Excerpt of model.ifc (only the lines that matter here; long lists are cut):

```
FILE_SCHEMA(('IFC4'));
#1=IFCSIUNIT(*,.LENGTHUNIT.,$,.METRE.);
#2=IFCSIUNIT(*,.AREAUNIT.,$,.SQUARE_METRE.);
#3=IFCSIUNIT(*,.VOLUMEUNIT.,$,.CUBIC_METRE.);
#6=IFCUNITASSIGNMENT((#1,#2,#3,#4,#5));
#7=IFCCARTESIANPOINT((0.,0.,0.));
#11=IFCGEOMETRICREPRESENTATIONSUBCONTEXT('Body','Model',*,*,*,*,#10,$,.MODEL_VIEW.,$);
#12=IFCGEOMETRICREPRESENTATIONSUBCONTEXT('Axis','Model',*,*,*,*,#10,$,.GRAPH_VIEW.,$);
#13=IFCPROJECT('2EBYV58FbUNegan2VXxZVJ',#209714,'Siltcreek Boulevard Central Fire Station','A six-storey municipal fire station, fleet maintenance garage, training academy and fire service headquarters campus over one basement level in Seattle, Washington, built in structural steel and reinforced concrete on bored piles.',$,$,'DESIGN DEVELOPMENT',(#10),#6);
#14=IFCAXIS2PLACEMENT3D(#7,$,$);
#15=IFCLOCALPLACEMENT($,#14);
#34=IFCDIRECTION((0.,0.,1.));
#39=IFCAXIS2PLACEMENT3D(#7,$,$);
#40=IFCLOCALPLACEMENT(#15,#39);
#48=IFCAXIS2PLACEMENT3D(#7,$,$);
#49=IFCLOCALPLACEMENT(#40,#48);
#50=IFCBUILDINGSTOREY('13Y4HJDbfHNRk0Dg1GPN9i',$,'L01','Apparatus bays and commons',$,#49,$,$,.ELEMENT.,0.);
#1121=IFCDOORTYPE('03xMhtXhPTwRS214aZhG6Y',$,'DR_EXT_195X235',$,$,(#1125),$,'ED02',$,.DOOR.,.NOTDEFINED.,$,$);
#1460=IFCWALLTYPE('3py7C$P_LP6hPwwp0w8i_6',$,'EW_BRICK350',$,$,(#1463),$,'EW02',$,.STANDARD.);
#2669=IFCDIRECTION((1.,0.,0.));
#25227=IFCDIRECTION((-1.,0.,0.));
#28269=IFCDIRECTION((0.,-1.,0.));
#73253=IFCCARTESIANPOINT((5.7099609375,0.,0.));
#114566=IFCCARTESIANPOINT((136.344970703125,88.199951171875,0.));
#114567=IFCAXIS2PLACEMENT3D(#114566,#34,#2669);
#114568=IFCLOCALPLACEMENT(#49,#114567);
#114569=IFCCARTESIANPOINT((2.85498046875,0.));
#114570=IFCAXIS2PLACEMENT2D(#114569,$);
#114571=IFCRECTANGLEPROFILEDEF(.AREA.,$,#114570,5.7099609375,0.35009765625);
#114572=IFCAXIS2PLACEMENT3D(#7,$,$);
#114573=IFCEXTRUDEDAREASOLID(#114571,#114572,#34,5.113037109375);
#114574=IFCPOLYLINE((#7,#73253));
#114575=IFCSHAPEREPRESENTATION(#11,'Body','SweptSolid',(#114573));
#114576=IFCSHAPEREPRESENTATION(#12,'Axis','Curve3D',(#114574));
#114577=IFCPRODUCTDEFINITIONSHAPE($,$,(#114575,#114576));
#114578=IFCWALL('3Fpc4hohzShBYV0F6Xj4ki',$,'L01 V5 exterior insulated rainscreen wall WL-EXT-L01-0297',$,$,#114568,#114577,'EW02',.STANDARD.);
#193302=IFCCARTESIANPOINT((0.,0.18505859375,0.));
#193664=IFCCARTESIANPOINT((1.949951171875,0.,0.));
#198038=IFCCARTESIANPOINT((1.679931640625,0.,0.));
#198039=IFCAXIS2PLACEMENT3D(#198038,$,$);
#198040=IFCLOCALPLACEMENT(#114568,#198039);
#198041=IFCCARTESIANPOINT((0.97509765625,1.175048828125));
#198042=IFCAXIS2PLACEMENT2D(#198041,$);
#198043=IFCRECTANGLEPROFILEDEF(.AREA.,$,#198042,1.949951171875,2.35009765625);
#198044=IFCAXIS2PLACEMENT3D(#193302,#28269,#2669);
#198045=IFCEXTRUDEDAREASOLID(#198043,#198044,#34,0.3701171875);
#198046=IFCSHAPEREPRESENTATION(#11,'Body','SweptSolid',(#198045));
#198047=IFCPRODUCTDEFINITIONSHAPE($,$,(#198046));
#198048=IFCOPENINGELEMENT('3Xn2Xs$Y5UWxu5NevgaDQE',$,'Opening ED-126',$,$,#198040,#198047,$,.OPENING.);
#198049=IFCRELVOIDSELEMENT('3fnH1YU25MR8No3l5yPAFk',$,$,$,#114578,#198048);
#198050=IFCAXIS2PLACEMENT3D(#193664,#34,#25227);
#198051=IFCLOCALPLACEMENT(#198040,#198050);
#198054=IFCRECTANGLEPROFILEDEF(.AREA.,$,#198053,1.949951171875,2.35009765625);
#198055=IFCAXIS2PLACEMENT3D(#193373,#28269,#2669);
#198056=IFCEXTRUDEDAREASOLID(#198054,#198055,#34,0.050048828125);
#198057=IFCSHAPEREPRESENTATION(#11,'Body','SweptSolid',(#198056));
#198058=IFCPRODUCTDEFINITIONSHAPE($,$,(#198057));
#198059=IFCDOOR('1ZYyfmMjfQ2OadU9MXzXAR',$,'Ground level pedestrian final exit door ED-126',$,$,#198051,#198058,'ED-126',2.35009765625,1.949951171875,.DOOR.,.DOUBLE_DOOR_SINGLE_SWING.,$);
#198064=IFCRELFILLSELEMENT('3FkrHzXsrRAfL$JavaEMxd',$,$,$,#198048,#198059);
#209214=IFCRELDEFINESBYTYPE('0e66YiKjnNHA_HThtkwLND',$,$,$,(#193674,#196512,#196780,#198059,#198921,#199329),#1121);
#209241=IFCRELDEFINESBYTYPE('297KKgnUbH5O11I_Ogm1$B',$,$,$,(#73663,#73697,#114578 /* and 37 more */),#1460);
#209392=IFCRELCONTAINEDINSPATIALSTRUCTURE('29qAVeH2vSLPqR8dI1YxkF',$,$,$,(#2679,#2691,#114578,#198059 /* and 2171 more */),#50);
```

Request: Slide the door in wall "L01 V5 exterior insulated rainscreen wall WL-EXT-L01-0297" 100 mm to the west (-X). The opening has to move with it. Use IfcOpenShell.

```python
import ifcopenshell
import ifcopenshell.api.geometry
import ifcopenshell.util.placement

model = ifcopenshell.open("model.ifc")

door = model.by_guid("1ZYyfmMjfQ2OadU9MXzXAR")
opening = door.FillsVoids[0].RelatingOpeningElement
wall = opening.VoidsElements[0].RelatingBuildingElement

wall_matrix = ifcopenshell.util.placement.get_local_placement(wall.ObjectPlacement)
shift = wall_matrix[:3, 0] * -0.1
before = ifcopenshell.util.placement.get_local_placement(door.ObjectPlacement)[:3, 3].copy()

# The door is placed relative to its opening, so it follows when the opening moves.
matrix = ifcopenshell.util.placement.get_local_placement(opening.ObjectPlacement)
matrix[:3, 3] += shift
ifcopenshell.api.geometry.edit_object_placement(
    model, product=opening, matrix=matrix, is_si=False, should_transform_children=True
)

after = ifcopenshell.util.placement.get_local_placement(door.ObjectPlacement)[:3, 3]
print("door moved by", (after - before).round(3) + 0.0)

model.write("model-out.ifc")
```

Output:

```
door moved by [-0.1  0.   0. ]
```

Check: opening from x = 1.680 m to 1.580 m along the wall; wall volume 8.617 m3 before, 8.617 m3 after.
